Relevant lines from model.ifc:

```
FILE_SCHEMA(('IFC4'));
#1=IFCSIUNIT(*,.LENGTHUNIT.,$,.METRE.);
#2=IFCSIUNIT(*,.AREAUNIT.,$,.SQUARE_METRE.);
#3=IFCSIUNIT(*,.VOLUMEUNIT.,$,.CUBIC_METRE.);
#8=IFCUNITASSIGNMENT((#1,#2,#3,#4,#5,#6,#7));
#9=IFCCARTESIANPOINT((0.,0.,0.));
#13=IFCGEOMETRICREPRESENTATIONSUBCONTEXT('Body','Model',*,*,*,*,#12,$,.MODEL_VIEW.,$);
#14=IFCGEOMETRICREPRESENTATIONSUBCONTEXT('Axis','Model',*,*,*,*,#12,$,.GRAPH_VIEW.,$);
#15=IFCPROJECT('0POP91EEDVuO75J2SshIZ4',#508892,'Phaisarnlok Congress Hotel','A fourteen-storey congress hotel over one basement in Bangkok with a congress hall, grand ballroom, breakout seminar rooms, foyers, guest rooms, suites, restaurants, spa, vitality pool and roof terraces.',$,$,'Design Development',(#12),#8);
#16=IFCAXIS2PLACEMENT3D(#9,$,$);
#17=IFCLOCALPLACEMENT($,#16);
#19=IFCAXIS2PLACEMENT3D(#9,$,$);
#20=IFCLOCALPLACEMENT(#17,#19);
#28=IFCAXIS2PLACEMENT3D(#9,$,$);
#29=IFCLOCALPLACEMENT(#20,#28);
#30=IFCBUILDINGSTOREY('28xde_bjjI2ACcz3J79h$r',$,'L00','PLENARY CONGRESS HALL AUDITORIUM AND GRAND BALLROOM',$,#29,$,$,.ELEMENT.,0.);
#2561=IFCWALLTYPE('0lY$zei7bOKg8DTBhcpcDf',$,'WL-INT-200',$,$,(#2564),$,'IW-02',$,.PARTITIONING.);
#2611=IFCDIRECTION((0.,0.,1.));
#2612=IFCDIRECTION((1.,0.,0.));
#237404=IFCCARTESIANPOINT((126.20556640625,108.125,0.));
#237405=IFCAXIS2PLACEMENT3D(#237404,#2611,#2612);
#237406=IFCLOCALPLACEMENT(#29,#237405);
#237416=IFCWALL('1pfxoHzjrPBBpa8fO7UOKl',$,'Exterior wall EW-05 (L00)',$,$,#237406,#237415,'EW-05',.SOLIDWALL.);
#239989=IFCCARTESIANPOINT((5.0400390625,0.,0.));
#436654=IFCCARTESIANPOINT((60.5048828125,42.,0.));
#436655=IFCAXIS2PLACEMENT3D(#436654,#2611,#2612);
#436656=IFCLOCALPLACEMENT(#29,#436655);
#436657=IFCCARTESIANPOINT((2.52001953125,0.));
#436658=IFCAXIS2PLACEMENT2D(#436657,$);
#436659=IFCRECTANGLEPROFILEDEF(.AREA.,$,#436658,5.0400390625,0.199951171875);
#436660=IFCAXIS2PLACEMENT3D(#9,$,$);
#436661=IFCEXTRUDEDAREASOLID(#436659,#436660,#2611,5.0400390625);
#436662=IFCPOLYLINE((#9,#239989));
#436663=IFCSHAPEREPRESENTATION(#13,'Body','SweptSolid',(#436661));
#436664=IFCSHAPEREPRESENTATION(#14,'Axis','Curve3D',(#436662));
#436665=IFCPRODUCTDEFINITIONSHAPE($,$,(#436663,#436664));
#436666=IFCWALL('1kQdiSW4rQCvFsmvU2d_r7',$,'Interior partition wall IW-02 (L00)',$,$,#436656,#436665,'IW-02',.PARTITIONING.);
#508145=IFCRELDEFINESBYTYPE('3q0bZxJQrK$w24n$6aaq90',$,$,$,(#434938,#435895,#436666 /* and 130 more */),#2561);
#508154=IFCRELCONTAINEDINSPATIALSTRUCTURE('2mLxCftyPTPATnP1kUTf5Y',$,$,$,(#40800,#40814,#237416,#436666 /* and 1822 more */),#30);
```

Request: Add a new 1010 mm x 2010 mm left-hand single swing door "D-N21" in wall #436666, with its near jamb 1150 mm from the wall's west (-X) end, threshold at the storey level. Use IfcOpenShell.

```python
import numpy as np
import ifcopenshell
import ifcopenshell.api.feature
import ifcopenshell.api.geometry
import ifcopenshell.api.root
import ifcopenshell.api.spatial
import ifcopenshell.geom
import ifcopenshell.util.element
import ifcopenshell.util.placement
import ifcopenshell.util.representation
import ifcopenshell.util.shape
import ifcopenshell.util.unit

model = ifcopenshell.open("model.ifc")
unit_scale = ifcopenshell.util.unit.calculate_unit_scale(model)
settings = ifcopenshell.geom.settings()


def volume(element):
    """Net volume in cubic metres, openings subtracted."""
    shape = ifcopenshell.geom.create_shape(settings, element)
    return ifcopenshell.util.shape.get_volume(shape.geometry)


wall = model.by_id(436666)
storey = ifcopenshell.util.element.get_container(wall, ifc_class="IfcBuildingStorey")
context = ifcopenshell.util.representation.get_context(model, "Model", "Body", "MODEL_VIEW")
before = volume(wall)

width, height, from_end, sill = 1.01, 2.01, 1.15, 0.0  # metres

# The wall runs along its own X axis, and the end named is its -X end.
wall_shape = ifcopenshell.geom.create_shape(settings, wall)
x, y, z = ifcopenshell.util.shape.get_vertices(wall_shape.geometry).T
start = x.min() + from_end
face, thickness = float(y.min()), float(y.max() - y.min())
wall_matrix = ifcopenshell.util.placement.get_local_placement(wall.ObjectPlacement)
level = ifcopenshell.util.placement.get_local_placement(storey.ObjectPlacement)[2, 3]


def in_wall(x, y):
    """Placement at x, y metres in the wall's axes, at sill height."""
    matrix = wall_matrix.copy()
    matrix[:, 3] = wall_matrix @ np.array([x / unit_scale, y / unit_scale, 0.0, 1.0])
    matrix[2, 3] = level + sill / unit_scale
    return matrix


# Opening: a box that overshoots both wall faces by 50 mm.
opening = ifcopenshell.api.root.create_entity(model, ifc_class="IfcOpeningElement", predefined_type="OPENING")
box = ifcopenshell.api.geometry.add_wall_representation(
    model, context=context, length=width, height=height, thickness=thickness + 0.1
)
ifcopenshell.api.geometry.assign_representation(model, product=opening, representation=box)
ifcopenshell.api.geometry.edit_object_placement(model, product=opening, matrix=in_wall(start, face - 0.05), is_si=False)
ifcopenshell.api.feature.add_feature(model, feature=opening, element=wall)

door = ifcopenshell.api.root.create_entity(model, ifc_class="IfcDoor", name="D-N21", predefined_type="DOOR")
door.OverallWidth, door.OverallHeight = width / unit_scale, height / unit_scale
door.OperationType = "SINGLE_SWING_LEFT"
body = ifcopenshell.api.geometry.add_door_representation(
    model,
    context=context,
    overall_width=door.OverallWidth,
    overall_height=door.OverallHeight,
    operation_type="SINGLE_SWING_LEFT",
    lining_properties={"LiningDepth": thickness / unit_scale, "ThresholdDepth": thickness / unit_scale},
)
ifcopenshell.api.geometry.assign_representation(model, product=door, representation=body)
ifcopenshell.api.spatial.assign_container(model, products=[door], relating_structure=storey)
ifcopenshell.api.feature.add_filling(model, opening=opening, element=door)

# The lining spans the wall, so the door starts at the wall face.
ifcopenshell.api.geometry.edit_object_placement(model, product=door, matrix=in_wall(start, face), is_si=False)

after = volume(wall)

print(f"wall volume {before:.3f} -> {after:.3f} m3")

model.write("model_updated.ifc")
```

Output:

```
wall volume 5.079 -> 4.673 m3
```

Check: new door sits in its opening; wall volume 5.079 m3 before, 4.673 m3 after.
